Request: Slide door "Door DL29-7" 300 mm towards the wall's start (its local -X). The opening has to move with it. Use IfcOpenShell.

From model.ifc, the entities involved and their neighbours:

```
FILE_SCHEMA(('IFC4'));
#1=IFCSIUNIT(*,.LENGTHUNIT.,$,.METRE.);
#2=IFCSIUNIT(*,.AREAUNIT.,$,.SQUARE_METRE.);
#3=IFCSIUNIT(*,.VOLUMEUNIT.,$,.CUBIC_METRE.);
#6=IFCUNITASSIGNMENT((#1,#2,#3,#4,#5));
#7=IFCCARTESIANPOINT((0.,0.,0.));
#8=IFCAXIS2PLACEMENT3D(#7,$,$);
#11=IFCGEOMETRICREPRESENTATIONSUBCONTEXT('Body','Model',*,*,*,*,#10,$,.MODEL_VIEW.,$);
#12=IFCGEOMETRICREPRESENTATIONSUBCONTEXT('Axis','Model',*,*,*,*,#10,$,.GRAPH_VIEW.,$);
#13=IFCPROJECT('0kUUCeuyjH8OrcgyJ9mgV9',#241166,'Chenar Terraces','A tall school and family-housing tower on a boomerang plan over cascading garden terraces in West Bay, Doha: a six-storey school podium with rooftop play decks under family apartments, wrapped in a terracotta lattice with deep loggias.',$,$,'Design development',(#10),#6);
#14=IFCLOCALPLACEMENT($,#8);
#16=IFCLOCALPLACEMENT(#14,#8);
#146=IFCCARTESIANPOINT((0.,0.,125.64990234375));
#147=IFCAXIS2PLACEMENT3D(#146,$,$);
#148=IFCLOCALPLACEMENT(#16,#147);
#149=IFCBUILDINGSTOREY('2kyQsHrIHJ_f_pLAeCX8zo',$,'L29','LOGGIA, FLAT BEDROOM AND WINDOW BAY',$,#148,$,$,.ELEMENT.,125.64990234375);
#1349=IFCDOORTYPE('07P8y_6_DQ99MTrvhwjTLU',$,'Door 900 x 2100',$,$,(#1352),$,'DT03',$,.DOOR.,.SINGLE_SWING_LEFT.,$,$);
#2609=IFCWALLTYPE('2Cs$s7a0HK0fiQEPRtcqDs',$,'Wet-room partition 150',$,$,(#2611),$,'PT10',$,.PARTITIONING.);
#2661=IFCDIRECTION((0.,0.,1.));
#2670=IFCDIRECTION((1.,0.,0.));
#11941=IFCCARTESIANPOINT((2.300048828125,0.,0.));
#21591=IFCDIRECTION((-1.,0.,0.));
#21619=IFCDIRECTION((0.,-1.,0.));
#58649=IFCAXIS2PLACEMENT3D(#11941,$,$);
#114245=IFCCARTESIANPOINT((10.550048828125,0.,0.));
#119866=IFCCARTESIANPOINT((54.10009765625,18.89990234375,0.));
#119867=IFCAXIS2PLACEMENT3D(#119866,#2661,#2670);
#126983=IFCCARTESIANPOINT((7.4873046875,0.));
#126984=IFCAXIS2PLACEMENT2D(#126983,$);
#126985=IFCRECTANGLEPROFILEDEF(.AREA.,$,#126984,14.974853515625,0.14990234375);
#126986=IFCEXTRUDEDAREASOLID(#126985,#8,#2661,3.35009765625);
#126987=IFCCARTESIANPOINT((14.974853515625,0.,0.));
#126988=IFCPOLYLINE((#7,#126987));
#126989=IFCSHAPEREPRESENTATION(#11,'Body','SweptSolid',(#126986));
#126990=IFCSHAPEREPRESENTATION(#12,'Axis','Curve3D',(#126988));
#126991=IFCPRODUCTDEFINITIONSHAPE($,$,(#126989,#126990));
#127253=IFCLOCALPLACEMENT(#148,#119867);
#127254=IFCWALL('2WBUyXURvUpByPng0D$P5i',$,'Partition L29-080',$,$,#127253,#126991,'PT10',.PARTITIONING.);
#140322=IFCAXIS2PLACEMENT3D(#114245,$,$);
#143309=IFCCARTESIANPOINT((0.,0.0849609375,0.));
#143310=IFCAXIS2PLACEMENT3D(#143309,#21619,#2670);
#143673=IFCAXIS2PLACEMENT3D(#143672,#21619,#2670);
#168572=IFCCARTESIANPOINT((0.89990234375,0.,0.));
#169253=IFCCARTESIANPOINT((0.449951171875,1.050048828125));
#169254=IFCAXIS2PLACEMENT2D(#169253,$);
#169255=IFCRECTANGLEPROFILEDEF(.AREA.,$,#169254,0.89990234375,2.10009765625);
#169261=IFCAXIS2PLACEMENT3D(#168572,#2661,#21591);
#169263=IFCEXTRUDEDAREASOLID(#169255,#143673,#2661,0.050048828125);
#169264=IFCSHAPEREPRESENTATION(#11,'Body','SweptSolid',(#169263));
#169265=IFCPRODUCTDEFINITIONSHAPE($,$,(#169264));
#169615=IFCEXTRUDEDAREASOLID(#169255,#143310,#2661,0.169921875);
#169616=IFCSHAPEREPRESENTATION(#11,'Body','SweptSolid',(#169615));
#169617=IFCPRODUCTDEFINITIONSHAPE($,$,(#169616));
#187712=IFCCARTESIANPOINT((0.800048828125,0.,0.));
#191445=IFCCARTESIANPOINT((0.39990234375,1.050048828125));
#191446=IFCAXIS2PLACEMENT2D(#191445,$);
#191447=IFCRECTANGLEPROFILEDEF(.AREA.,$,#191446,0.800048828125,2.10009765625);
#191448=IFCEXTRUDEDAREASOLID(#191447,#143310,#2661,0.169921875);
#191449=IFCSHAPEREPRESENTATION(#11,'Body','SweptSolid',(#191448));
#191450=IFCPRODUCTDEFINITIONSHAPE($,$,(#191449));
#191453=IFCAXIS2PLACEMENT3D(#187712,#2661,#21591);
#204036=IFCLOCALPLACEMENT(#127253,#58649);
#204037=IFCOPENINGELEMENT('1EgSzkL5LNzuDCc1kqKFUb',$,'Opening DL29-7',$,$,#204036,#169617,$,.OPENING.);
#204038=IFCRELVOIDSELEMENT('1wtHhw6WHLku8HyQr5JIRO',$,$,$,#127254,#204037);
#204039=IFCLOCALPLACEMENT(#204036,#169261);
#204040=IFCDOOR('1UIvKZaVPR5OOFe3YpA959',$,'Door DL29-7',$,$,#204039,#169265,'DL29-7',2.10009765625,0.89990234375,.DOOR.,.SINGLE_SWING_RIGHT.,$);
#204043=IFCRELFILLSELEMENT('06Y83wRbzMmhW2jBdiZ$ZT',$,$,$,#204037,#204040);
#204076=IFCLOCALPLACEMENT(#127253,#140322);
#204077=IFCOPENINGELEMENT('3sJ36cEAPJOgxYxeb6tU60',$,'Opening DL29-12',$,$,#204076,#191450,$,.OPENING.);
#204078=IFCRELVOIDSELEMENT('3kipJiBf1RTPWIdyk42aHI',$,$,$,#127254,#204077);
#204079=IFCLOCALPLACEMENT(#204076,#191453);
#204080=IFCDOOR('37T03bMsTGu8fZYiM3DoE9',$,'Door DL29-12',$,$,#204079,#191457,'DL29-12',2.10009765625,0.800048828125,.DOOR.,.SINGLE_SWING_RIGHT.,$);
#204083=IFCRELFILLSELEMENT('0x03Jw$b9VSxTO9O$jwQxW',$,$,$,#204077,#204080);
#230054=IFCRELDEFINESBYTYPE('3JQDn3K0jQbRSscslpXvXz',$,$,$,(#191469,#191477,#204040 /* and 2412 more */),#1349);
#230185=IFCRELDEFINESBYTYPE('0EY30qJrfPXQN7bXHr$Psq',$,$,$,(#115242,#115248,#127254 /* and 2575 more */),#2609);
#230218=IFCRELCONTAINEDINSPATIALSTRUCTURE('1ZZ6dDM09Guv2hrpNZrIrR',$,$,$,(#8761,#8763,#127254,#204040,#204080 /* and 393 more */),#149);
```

```python
import ifcopenshell
import ifcopenshell.api.geometry
import ifcopenshell.util.placement

model = ifcopenshell.open("model.ifc")

door = model.by_guid("1UIvKZaVPR5OOFe3YpA959")
opening = door.FillsVoids[0].RelatingOpeningElement
wall = opening.VoidsElements[0].RelatingBuildingElement

wall_matrix = ifcopenshell.util.placement.get_local_placement(wall.ObjectPlacement)
shift = wall_matrix[:3, 0] * -0.3
before = ifcopenshell.util.placement.get_local_placement(door.ObjectPlacement)[:3, 3].copy()

# The door is placed relative to its opening, so it follows when the opening moves.
matrix = ifcopenshell.util.placement.get_local_placement(opening.ObjectPlacement)
matrix[:3, 3] += shift
ifcopenshell.api.geometry.edit_object_placement(
    model, product=opening, matrix=matrix, is_si=False, should_transform_children=True
)

after = ifcopenshell.util.placement.get_local_placement(door.ObjectPlacement)[:3, 3]
print("door moved by", (after - before).round(3) + 0.0)

model.write("model-out.ifc")
```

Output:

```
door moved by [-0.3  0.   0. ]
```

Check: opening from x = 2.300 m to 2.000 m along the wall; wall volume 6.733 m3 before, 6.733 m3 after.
